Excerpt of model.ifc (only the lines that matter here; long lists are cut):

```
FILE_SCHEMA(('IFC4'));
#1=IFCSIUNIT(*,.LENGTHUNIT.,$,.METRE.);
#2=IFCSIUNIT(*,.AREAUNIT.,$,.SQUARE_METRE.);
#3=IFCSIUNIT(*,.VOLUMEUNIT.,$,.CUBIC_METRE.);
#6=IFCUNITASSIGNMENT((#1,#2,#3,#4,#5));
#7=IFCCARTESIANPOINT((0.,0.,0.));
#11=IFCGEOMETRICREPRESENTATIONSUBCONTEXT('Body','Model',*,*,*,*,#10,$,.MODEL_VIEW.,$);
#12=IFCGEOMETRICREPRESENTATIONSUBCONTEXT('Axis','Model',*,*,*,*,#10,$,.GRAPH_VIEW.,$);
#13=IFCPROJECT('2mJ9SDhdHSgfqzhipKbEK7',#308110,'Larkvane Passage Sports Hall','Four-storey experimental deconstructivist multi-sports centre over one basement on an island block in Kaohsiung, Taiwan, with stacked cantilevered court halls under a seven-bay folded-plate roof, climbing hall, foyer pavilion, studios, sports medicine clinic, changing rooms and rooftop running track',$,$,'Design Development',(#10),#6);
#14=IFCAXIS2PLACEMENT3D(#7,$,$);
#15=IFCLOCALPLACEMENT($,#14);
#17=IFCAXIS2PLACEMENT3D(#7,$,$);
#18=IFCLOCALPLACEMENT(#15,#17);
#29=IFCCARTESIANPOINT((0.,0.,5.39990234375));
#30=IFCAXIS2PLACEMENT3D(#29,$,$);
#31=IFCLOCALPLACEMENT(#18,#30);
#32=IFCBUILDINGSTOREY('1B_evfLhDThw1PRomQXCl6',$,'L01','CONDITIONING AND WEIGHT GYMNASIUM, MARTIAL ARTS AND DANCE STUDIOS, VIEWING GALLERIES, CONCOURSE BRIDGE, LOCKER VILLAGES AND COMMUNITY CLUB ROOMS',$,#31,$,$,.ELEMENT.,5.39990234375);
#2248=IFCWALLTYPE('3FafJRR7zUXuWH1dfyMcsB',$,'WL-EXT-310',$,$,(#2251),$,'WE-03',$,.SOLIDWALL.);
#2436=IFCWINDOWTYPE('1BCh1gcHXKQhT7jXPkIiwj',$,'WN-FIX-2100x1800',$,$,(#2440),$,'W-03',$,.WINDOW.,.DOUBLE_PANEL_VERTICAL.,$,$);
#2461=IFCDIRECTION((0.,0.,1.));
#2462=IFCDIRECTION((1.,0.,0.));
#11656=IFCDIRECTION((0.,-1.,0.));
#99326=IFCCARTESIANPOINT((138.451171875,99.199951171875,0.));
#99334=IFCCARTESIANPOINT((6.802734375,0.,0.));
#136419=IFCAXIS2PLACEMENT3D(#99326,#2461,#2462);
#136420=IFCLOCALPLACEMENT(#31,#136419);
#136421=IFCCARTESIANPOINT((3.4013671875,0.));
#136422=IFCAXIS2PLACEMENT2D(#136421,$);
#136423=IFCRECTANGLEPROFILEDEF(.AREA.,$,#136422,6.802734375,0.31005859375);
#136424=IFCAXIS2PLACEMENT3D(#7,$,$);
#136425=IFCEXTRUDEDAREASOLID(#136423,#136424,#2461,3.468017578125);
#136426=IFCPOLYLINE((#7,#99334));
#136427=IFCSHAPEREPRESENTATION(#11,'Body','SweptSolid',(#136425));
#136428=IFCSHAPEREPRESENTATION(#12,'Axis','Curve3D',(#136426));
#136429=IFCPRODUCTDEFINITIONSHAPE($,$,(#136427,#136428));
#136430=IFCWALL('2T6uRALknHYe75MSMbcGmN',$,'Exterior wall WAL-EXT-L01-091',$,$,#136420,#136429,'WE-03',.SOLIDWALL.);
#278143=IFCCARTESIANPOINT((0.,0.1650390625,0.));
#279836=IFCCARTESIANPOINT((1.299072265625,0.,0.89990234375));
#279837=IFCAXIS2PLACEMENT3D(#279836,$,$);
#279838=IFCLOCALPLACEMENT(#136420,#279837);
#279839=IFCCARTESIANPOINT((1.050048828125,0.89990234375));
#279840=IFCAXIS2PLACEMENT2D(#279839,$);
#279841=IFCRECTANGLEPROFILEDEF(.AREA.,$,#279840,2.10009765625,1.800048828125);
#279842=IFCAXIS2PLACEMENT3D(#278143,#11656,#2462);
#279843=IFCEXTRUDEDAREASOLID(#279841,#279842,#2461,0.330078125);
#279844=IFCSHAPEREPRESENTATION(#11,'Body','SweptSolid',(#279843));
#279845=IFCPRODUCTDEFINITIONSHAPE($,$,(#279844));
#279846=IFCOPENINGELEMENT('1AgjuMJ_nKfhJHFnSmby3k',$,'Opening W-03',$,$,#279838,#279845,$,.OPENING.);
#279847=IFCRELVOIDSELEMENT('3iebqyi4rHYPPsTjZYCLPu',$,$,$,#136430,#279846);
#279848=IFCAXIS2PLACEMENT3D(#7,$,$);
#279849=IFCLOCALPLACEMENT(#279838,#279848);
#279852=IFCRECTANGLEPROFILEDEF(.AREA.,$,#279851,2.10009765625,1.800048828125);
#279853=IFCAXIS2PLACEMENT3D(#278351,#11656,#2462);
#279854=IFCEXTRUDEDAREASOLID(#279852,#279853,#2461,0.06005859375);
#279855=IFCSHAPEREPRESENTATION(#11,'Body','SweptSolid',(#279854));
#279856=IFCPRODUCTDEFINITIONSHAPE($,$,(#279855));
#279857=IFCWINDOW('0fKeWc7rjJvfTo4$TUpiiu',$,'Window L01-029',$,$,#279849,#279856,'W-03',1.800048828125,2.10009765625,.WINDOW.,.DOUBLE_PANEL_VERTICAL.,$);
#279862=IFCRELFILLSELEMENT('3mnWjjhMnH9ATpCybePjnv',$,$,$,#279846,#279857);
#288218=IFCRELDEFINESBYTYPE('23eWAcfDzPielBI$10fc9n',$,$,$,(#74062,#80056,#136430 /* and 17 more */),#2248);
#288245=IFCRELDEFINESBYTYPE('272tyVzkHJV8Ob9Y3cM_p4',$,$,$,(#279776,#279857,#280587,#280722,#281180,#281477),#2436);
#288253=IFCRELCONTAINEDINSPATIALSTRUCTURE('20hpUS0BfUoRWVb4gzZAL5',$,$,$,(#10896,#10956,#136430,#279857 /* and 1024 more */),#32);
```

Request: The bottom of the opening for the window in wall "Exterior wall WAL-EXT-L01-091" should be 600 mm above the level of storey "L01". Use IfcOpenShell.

```python
import numpy as np
import ifcopenshell
import ifcopenshell.api.geometry
import ifcopenshell.geom
import ifcopenshell.util.element
import ifcopenshell.util.placement
import ifcopenshell.util.shape
import ifcopenshell.util.unit

model = ifcopenshell.open("model.ifc")
unit_scale = ifcopenshell.util.unit.calculate_unit_scale(model)

window = model.by_guid("0fKeWc7rjJvfTo4$TUpiiu")
opening = window.FillsVoids[0].RelatingOpeningElement
storey = ifcopenshell.util.element.get_container(window, ifc_class="IfcBuildingStorey")
level = ifcopenshell.util.placement.get_local_placement(storey.ObjectPlacement)[2, 3]

# The opening's origin need not be at the sill, so measure its lowest point.
shape = ifcopenshell.geom.create_shape(ifcopenshell.geom.settings(), opening)
bottom = ifcopenshell.util.shape.get_shape_bottom_elevation(shape, shape.geometry) / unit_scale
dz = level + 0.6 / unit_scale - bottom

shift = np.array([0.0, 0.0, dz])
# The window is placed relative to its opening, so it follows when the opening moves.
matrix = ifcopenshell.util.placement.get_local_placement(opening.ObjectPlacement)
matrix[:3, 3] += shift
ifcopenshell.api.geometry.edit_object_placement(
    model, product=opening, matrix=matrix, is_si=False, should_transform_children=True
)

print(f"moved by {dz * unit_scale:+.3f} m")

model.write("model_rev.ifc")
```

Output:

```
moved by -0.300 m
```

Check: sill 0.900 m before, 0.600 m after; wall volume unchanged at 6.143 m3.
